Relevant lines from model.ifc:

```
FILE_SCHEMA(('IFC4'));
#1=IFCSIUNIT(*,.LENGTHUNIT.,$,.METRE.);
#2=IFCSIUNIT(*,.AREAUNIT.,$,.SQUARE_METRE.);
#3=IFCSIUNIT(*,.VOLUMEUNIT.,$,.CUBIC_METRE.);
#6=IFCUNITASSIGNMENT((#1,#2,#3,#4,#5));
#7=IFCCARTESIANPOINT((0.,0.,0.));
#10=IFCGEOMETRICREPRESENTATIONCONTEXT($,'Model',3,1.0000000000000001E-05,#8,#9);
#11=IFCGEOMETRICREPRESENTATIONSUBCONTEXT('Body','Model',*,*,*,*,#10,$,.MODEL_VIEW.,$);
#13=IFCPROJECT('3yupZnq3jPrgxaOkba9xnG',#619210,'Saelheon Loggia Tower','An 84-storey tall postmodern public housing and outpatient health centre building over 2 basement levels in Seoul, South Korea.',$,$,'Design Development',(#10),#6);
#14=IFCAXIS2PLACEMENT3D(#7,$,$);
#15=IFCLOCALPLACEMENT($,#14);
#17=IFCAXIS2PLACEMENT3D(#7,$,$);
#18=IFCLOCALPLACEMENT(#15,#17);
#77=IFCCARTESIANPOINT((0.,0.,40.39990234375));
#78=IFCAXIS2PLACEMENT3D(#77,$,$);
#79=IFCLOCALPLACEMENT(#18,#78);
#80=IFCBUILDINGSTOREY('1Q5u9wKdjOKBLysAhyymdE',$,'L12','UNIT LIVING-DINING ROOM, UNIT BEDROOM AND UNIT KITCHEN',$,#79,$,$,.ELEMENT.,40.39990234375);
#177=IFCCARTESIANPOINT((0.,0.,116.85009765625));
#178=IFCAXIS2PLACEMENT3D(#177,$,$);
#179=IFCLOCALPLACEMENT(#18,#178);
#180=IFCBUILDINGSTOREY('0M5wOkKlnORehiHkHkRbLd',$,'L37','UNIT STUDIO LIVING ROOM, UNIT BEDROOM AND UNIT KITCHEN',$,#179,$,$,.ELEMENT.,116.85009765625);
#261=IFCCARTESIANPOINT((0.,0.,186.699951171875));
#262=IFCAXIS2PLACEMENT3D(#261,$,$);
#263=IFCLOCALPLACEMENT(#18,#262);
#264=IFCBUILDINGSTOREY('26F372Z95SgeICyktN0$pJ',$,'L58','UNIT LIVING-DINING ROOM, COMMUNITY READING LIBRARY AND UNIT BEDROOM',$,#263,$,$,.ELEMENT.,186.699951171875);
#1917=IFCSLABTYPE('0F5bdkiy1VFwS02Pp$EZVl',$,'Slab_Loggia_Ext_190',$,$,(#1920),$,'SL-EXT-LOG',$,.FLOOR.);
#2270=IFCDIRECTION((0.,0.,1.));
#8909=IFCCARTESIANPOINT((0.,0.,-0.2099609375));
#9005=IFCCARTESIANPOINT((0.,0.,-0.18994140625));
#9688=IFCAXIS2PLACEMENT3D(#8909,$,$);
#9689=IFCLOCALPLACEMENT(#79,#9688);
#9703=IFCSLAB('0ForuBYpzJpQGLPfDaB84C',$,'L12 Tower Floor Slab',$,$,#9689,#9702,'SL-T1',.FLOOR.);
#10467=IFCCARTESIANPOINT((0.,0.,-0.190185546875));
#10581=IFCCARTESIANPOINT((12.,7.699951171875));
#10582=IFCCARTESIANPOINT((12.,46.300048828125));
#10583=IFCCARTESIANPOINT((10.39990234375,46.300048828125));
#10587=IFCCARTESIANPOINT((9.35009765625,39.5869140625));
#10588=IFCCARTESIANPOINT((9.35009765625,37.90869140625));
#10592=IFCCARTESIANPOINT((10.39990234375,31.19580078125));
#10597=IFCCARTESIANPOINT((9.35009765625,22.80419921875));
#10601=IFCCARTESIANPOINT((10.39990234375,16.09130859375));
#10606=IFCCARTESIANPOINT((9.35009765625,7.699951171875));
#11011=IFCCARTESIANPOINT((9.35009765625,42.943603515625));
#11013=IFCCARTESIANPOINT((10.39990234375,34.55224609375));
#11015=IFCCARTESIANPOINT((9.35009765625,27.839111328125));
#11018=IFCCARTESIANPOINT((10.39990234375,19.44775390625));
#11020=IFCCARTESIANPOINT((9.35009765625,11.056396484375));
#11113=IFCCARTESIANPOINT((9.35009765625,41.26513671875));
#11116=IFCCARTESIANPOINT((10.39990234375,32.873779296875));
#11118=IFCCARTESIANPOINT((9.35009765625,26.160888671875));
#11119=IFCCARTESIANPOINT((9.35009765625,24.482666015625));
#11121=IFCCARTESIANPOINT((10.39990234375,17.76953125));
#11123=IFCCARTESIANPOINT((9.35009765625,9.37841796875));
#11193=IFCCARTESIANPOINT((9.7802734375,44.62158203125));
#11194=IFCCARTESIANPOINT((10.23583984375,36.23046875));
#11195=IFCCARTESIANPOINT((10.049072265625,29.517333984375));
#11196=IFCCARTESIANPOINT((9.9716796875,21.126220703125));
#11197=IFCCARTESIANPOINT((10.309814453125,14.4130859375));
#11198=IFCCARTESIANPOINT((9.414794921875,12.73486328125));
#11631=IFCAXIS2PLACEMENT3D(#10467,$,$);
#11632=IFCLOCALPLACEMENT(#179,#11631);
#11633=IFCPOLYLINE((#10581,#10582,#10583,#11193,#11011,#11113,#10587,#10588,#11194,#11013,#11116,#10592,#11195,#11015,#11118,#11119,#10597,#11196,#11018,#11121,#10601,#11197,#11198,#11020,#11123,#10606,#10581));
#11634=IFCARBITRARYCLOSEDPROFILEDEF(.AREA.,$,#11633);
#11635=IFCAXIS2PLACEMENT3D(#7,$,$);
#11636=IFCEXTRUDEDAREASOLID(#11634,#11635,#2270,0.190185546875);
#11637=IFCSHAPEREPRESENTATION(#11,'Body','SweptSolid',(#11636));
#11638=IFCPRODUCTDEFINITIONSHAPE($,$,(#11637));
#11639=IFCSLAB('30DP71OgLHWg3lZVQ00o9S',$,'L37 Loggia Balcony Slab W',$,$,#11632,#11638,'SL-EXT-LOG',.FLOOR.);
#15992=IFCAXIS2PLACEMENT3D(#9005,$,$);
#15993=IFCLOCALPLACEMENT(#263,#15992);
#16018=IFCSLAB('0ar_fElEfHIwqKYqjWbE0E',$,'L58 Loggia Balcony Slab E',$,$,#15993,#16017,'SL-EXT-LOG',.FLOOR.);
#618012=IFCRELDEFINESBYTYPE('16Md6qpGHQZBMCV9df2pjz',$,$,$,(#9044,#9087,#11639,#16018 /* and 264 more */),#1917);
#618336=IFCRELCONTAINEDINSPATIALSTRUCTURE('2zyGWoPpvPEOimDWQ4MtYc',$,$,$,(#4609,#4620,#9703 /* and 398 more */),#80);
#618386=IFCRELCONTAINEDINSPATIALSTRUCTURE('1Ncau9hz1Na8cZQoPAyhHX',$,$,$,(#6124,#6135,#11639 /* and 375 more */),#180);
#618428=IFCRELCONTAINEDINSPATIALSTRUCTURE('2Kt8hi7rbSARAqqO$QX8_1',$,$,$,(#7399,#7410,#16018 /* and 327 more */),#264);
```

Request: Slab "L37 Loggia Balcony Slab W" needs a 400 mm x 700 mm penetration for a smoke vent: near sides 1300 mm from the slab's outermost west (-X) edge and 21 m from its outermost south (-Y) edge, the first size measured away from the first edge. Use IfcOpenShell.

```python
import numpy as np
import ifcopenshell
import ifcopenshell.api.feature
import ifcopenshell.api.geometry
import ifcopenshell.api.root
import ifcopenshell.geom
import ifcopenshell.util.placement
import ifcopenshell.util.representation
import ifcopenshell.util.shape
import ifcopenshell.util.unit

model = ifcopenshell.open("model.ifc")
unit_scale = ifcopenshell.util.unit.calculate_unit_scale(model)
settings = ifcopenshell.geom.settings()


def volume(element):
    """Net volume in cubic metres, openings subtracted."""
    shape = ifcopenshell.geom.create_shape(settings, element)
    return ifcopenshell.util.shape.get_volume(shape.geometry)


slab = model.by_id(11639)
before = volume(slab)

# Extent in the slab's own axes, in metres. The edges named are its -X and -Y sides.
slab_shape = ifcopenshell.geom.create_shape(settings, slab)
vertices = ifcopenshell.util.shape.get_vertices(slab_shape.geometry)
x_min, y_min, bottom = vertices.min(axis=0)
top = vertices[:, 2].max()

opening = ifcopenshell.api.root.create_entity(model, ifc_class="IfcOpeningElement", name="Smoke vent opening", predefined_type="OPENING")
context = ifcopenshell.util.representation.get_context(model, "Model", "Body", "MODEL_VIEW")
width, depth = 0.4, 0.7
outline = [(0.0, 0.0), (width, 0.0), (width, depth), (0.0, depth), (0.0, 0.0)]
# Overshoot both faces by 50 mm so the cut is clean.
shape = ifcopenshell.api.geometry.add_slab_representation(
    model, context=context, depth=top - bottom + 0.1, polyline=outline
)
ifcopenshell.api.geometry.assign_representation(model, product=opening, representation=shape)

matrix = ifcopenshell.util.placement.get_local_placement(slab.ObjectPlacement)
matrix[:, 3] = matrix @ np.append(np.array([x_min + 1.3, y_min + 21, bottom - 0.05]) / unit_scale, 1.0)
ifcopenshell.api.geometry.edit_object_placement(model, product=opening, matrix=matrix, is_si=False)
ifcopenshell.api.feature.add_feature(model, feature=opening, element=slab)

after = volume(slab)

print(f"slab volume {before:.3f} -> {after:.3f} m3")

model.write("model_edited.ifc")
```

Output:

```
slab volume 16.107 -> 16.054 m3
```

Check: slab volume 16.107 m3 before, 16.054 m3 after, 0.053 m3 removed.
